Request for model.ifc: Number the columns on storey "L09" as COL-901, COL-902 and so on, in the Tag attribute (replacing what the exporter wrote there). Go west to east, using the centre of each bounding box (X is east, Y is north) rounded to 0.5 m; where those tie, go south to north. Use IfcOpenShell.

First a look at what the model holds.

```python
import ifcopenshell
import ifcopenshell.util.element
import ifcopenshell.util.placement

model = ifcopenshell.open("model.ifc")
print(model.schema)
storey = next(s for s in model.by_type("IfcBuildingStorey") if s.Name == "L09")
columns = [e for e in ifcopenshell.util.element.get_decomposition(storey) if e.is_a("IfcColumn")]
for e in sorted(columns, key=lambda e: e.id()):
    origin = ifcopenshell.util.placement.get_local_placement(e.ObjectPlacement)[:3, 3]
    print(e.id(), e.Tag, e.Name, origin.round(2) + 0.0, sep=" | ")
```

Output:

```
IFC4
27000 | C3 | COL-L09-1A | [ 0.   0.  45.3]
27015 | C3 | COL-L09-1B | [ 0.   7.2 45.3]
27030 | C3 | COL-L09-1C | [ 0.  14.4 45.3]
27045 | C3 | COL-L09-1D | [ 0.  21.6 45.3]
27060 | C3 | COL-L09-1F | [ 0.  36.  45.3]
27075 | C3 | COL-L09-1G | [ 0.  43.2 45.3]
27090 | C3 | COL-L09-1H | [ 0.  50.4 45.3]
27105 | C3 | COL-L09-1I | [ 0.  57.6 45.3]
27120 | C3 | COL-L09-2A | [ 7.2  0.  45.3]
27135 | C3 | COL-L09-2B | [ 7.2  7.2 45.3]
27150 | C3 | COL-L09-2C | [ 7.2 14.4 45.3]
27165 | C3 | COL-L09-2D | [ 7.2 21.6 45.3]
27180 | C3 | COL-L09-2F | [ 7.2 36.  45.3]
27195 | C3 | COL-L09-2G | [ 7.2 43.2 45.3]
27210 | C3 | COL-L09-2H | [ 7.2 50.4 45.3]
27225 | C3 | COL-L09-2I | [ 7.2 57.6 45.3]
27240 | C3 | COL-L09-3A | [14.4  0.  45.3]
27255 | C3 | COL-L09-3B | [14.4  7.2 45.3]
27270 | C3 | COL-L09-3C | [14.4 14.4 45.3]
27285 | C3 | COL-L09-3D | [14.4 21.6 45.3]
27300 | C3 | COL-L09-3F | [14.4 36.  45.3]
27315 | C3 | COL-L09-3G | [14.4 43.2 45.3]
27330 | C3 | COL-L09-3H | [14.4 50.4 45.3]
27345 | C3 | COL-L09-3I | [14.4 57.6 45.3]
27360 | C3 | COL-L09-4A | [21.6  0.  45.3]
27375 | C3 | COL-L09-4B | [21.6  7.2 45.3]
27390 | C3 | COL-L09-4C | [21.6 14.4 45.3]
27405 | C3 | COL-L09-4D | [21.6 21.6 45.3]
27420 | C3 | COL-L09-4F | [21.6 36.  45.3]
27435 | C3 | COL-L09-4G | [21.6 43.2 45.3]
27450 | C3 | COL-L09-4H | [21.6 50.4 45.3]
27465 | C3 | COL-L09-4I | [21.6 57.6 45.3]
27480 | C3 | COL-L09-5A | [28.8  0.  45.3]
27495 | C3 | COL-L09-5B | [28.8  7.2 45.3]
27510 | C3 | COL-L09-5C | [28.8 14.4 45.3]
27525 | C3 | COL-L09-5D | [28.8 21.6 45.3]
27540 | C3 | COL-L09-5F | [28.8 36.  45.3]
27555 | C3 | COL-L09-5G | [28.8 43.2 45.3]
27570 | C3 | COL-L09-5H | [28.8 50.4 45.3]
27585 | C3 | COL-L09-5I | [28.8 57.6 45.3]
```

```python
import ifcopenshell
import ifcopenshell.geom
import ifcopenshell.util.element
import ifcopenshell.util.shape

model = ifcopenshell.open("model.ifc")
settings = ifcopenshell.geom.settings()
settings.set("use-world-coords", True)


def centre(element):
    shape = ifcopenshell.geom.create_shape(settings, element)
    return ifcopenshell.util.shape.get_bbox_centroid(shape.geometry)


storey = next(s for s in model.by_type("IfcBuildingStorey") if s.Name == "L09")
columns = [e for e in ifcopenshell.util.element.get_decomposition(storey) if e.is_a("IfcColumn")]

# Insertion points can sit at a corner or the storey origin, so sort by the geometry (in metres).
centres = {e: centre(e) for e in columns}
columns.sort(key=lambda e: (round(centres[e][0] / 0.5), centres[e][1]))

for i, e in enumerate(columns, start=1):
    number = f"COL-9{i:02d}"
    e.Tag = number
    print(e.id(), number)

model.write("model-out.ifc")
```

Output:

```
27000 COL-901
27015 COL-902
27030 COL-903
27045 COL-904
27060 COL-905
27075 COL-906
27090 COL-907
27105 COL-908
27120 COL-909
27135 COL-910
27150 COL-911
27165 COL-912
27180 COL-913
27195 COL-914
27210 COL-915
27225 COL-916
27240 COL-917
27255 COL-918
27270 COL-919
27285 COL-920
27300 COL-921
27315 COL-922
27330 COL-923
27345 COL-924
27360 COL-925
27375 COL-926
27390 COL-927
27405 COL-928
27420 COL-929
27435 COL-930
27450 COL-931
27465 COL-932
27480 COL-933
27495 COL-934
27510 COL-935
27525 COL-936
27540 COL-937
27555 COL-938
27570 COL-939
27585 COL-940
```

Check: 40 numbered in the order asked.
